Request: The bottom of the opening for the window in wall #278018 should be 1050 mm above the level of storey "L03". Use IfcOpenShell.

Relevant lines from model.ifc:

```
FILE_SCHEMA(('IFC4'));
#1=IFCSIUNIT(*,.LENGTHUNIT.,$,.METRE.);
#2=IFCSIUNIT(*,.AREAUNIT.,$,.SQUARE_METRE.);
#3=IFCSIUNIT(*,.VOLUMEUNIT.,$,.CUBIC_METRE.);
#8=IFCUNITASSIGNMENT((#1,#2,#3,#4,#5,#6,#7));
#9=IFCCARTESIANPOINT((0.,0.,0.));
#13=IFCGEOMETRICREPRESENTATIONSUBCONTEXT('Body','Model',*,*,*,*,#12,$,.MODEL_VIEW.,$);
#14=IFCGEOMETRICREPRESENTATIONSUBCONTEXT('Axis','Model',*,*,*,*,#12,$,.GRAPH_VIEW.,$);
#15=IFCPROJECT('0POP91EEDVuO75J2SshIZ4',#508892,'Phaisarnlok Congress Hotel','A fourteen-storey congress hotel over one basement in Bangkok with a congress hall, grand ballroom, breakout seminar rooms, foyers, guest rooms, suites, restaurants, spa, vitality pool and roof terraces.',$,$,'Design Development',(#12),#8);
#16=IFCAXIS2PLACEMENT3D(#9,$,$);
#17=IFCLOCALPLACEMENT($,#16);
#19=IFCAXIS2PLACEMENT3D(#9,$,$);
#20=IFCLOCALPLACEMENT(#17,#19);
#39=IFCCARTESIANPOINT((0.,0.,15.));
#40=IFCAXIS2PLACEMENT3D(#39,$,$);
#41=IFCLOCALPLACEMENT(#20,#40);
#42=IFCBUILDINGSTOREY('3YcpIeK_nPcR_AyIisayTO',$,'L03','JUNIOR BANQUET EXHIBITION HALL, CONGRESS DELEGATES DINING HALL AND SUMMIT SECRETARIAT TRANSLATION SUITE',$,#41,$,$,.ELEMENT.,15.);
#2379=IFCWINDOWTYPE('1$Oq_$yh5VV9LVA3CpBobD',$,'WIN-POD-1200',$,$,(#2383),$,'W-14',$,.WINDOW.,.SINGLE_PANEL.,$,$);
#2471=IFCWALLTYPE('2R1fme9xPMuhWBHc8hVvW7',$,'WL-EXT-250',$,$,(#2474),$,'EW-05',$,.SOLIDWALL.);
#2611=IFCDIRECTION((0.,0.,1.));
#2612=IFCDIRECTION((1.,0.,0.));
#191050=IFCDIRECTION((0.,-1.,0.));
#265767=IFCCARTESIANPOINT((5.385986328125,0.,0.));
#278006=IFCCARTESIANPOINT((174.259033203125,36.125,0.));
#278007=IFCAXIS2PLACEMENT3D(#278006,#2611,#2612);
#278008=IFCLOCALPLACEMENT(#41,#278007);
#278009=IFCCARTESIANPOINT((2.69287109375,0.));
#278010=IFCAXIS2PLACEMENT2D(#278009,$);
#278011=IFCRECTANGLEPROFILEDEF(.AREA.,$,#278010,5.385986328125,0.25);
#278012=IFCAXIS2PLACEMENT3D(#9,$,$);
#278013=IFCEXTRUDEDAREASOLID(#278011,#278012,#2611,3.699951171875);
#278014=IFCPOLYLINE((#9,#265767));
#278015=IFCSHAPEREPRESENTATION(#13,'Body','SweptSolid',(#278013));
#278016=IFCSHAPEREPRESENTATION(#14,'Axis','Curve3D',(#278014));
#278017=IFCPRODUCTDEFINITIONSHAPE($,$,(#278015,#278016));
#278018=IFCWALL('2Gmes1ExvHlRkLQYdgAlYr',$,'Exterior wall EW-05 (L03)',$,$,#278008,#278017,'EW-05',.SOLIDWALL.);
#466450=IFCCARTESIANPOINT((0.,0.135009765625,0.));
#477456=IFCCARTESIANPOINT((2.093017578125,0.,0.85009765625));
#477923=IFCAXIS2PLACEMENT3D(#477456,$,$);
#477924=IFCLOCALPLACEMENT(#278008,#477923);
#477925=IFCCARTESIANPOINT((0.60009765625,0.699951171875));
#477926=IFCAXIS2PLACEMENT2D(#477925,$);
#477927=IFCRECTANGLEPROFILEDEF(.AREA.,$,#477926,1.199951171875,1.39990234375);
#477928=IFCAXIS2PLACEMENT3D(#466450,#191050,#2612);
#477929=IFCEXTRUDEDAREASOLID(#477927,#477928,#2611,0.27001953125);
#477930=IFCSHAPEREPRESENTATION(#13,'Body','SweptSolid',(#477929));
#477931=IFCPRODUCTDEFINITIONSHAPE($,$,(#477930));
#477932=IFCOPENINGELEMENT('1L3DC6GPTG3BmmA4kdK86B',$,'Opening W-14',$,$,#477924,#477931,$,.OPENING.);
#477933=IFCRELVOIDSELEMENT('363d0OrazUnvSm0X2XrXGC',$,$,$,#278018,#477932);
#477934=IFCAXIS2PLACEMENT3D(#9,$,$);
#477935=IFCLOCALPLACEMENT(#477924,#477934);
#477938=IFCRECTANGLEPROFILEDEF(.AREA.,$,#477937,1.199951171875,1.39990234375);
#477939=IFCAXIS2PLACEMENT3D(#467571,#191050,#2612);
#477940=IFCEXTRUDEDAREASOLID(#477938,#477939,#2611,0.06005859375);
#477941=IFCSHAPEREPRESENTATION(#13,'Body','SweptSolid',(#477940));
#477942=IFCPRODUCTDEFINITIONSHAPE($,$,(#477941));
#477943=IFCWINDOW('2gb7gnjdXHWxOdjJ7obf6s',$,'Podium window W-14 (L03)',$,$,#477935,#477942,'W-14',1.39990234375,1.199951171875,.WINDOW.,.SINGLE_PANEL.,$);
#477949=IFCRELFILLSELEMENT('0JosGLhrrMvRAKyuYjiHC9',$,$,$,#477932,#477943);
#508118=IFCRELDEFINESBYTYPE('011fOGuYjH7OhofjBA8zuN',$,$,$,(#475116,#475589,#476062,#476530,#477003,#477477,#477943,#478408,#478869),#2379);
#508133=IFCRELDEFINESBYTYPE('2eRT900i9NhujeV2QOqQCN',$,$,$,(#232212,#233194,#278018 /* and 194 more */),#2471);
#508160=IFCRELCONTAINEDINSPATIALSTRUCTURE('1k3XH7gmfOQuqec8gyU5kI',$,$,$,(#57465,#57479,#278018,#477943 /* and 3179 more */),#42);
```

```python
import numpy as np
import ifcopenshell
import ifcopenshell.api.geometry
import ifcopenshell.geom
import ifcopenshell.util.element
import ifcopenshell.util.placement
import ifcopenshell.util.shape
import ifcopenshell.util.unit

model = ifcopenshell.open("model.ifc")
unit_scale = ifcopenshell.util.unit.calculate_unit_scale(model)

window = model.by_id(477943)
opening = window.FillsVoids[0].RelatingOpeningElement
storey = ifcopenshell.util.element.get_container(window, ifc_class="IfcBuildingStorey")
level = ifcopenshell.util.placement.get_local_placement(storey.ObjectPlacement)[2, 3]

# The opening's origin need not be at the sill, so measure its lowest point.
shape = ifcopenshell.geom.create_shape(ifcopenshell.geom.settings(), opening)
bottom = ifcopenshell.util.shape.get_shape_bottom_elevation(shape, shape.geometry) / unit_scale
dz = level + 1.05 / unit_scale - bottom

shift = np.array([0.0, 0.0, dz])
# The window is placed relative to its opening, so it follows when the opening moves.
matrix = ifcopenshell.util.placement.get_local_placement(opening.ObjectPlacement)
matrix[:3, 3] += shift
ifcopenshell.api.geometry.edit_object_placement(
    model, product=opening, matrix=matrix, is_si=False, should_transform_children=True
)

print(f"moved by {dz * unit_scale:+.3f} m")

model.write("model_edited.ifc")
```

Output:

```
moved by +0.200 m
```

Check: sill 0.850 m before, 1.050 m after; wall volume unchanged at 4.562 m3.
